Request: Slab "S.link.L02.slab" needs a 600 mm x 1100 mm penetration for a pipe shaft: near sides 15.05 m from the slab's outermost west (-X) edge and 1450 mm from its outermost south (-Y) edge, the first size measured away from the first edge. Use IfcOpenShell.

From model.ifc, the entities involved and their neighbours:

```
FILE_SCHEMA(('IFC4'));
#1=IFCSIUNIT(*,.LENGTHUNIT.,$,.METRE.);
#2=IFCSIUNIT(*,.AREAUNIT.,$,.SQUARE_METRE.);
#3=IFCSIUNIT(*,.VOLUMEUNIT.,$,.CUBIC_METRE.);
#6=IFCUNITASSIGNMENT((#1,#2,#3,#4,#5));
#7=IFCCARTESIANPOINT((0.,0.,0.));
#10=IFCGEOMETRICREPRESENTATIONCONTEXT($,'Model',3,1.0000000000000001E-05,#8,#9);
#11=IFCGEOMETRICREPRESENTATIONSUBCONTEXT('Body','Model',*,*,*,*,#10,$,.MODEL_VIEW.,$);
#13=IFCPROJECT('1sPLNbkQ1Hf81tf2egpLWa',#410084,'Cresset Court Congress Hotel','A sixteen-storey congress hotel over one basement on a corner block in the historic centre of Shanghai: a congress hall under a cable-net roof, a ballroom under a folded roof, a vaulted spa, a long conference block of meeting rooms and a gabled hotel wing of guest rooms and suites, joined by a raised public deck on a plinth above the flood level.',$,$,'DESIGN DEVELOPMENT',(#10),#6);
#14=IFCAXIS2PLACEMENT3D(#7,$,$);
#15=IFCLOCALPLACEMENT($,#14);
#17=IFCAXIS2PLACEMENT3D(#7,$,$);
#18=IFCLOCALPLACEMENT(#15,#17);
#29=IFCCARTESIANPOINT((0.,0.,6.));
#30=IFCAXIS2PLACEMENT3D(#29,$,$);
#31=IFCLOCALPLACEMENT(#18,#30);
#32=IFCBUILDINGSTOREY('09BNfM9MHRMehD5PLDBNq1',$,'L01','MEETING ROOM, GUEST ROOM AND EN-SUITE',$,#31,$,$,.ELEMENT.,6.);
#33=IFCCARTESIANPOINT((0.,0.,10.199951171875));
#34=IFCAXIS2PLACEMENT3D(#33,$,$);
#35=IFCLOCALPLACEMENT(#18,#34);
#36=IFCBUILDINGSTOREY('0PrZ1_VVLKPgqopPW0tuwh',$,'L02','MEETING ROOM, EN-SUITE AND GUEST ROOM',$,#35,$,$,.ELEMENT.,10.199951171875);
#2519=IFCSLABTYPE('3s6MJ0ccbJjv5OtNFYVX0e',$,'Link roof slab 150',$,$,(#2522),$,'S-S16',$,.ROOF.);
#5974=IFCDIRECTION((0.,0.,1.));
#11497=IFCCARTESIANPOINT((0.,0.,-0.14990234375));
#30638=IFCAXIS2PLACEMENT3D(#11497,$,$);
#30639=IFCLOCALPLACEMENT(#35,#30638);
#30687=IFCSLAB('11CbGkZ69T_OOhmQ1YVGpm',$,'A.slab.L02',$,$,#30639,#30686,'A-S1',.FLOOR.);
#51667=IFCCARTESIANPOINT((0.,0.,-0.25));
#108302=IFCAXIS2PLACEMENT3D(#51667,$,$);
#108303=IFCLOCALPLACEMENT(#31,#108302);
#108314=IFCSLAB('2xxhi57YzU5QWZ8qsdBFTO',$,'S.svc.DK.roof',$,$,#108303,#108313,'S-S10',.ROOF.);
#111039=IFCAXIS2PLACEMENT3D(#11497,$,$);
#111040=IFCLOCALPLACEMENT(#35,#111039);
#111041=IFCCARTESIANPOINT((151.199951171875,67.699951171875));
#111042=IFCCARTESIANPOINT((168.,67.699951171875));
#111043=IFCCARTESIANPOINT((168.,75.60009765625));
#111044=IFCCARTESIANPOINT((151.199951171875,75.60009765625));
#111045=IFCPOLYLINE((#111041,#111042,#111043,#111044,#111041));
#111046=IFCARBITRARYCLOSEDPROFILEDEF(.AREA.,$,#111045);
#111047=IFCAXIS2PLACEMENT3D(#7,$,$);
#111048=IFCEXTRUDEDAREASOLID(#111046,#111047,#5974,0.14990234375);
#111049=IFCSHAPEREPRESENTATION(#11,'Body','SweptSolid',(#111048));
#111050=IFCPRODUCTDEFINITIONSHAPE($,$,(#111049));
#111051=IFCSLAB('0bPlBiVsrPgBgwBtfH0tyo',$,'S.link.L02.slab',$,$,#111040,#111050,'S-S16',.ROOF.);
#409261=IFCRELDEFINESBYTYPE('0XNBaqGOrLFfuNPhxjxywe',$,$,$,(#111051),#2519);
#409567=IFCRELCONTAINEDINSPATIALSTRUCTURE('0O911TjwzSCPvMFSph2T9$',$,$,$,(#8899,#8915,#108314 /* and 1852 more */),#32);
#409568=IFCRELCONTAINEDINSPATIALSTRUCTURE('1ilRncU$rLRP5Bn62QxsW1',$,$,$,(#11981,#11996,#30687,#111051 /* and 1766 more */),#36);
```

```python
import numpy as np
import ifcopenshell
import ifcopenshell.api.feature
import ifcopenshell.api.geometry
import ifcopenshell.api.root
import ifcopenshell.geom
import ifcopenshell.util.placement
import ifcopenshell.util.representation
import ifcopenshell.util.shape
import ifcopenshell.util.unit

model = ifcopenshell.open("model.ifc")
unit_scale = ifcopenshell.util.unit.calculate_unit_scale(model)
settings = ifcopenshell.geom.settings()


def volume(element):
    """Net volume in cubic metres, openings subtracted."""
    shape = ifcopenshell.geom.create_shape(settings, element)
    return ifcopenshell.util.shape.get_volume(shape.geometry)


slab = model.by_id(111051)
before = volume(slab)

# Extent in the slab's own axes, in metres. The edges named are its -X and -Y sides.
slab_shape = ifcopenshell.geom.create_shape(settings, slab)
vertices = ifcopenshell.util.shape.get_vertices(slab_shape.geometry)
x_min, y_min, bottom = vertices.min(axis=0)
top = vertices[:, 2].max()

opening = ifcopenshell.api.root.create_entity(model, ifc_class="IfcOpeningElement", name="Pipe shaft opening", predefined_type="OPENING")
context = ifcopenshell.util.representation.get_context(model, "Model", "Body", "MODEL_VIEW")
width, depth = 0.6, 1.1
outline = [(0.0, 0.0), (width, 0.0), (width, depth), (0.0, depth), (0.0, 0.0)]
# Overshoot both faces by 50 mm so the cut is clean.
shape = ifcopenshell.api.geometry.add_slab_representation(
    model, context=context, depth=top - bottom + 0.1, polyline=outline
)
ifcopenshell.api.geometry.assign_representation(model, product=opening, representation=shape)

matrix = ifcopenshell.util.placement.get_local_placement(slab.ObjectPlacement)
matrix[:, 3] = matrix @ np.append(np.array([x_min + 15.05, y_min + 1.45, bottom - 0.05]) / unit_scale, 1.0)
ifcopenshell.api.geometry.edit_object_placement(model, product=opening, matrix=matrix, is_si=False)
ifcopenshell.api.feature.add_feature(model, feature=opening, element=slab)

after = volume(slab)

print(f"slab volume {before:.3f} -> {after:.3f} m3")

model.write("model_rev.ifc")
```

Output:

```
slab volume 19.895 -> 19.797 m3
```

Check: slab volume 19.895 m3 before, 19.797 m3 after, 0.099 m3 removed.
